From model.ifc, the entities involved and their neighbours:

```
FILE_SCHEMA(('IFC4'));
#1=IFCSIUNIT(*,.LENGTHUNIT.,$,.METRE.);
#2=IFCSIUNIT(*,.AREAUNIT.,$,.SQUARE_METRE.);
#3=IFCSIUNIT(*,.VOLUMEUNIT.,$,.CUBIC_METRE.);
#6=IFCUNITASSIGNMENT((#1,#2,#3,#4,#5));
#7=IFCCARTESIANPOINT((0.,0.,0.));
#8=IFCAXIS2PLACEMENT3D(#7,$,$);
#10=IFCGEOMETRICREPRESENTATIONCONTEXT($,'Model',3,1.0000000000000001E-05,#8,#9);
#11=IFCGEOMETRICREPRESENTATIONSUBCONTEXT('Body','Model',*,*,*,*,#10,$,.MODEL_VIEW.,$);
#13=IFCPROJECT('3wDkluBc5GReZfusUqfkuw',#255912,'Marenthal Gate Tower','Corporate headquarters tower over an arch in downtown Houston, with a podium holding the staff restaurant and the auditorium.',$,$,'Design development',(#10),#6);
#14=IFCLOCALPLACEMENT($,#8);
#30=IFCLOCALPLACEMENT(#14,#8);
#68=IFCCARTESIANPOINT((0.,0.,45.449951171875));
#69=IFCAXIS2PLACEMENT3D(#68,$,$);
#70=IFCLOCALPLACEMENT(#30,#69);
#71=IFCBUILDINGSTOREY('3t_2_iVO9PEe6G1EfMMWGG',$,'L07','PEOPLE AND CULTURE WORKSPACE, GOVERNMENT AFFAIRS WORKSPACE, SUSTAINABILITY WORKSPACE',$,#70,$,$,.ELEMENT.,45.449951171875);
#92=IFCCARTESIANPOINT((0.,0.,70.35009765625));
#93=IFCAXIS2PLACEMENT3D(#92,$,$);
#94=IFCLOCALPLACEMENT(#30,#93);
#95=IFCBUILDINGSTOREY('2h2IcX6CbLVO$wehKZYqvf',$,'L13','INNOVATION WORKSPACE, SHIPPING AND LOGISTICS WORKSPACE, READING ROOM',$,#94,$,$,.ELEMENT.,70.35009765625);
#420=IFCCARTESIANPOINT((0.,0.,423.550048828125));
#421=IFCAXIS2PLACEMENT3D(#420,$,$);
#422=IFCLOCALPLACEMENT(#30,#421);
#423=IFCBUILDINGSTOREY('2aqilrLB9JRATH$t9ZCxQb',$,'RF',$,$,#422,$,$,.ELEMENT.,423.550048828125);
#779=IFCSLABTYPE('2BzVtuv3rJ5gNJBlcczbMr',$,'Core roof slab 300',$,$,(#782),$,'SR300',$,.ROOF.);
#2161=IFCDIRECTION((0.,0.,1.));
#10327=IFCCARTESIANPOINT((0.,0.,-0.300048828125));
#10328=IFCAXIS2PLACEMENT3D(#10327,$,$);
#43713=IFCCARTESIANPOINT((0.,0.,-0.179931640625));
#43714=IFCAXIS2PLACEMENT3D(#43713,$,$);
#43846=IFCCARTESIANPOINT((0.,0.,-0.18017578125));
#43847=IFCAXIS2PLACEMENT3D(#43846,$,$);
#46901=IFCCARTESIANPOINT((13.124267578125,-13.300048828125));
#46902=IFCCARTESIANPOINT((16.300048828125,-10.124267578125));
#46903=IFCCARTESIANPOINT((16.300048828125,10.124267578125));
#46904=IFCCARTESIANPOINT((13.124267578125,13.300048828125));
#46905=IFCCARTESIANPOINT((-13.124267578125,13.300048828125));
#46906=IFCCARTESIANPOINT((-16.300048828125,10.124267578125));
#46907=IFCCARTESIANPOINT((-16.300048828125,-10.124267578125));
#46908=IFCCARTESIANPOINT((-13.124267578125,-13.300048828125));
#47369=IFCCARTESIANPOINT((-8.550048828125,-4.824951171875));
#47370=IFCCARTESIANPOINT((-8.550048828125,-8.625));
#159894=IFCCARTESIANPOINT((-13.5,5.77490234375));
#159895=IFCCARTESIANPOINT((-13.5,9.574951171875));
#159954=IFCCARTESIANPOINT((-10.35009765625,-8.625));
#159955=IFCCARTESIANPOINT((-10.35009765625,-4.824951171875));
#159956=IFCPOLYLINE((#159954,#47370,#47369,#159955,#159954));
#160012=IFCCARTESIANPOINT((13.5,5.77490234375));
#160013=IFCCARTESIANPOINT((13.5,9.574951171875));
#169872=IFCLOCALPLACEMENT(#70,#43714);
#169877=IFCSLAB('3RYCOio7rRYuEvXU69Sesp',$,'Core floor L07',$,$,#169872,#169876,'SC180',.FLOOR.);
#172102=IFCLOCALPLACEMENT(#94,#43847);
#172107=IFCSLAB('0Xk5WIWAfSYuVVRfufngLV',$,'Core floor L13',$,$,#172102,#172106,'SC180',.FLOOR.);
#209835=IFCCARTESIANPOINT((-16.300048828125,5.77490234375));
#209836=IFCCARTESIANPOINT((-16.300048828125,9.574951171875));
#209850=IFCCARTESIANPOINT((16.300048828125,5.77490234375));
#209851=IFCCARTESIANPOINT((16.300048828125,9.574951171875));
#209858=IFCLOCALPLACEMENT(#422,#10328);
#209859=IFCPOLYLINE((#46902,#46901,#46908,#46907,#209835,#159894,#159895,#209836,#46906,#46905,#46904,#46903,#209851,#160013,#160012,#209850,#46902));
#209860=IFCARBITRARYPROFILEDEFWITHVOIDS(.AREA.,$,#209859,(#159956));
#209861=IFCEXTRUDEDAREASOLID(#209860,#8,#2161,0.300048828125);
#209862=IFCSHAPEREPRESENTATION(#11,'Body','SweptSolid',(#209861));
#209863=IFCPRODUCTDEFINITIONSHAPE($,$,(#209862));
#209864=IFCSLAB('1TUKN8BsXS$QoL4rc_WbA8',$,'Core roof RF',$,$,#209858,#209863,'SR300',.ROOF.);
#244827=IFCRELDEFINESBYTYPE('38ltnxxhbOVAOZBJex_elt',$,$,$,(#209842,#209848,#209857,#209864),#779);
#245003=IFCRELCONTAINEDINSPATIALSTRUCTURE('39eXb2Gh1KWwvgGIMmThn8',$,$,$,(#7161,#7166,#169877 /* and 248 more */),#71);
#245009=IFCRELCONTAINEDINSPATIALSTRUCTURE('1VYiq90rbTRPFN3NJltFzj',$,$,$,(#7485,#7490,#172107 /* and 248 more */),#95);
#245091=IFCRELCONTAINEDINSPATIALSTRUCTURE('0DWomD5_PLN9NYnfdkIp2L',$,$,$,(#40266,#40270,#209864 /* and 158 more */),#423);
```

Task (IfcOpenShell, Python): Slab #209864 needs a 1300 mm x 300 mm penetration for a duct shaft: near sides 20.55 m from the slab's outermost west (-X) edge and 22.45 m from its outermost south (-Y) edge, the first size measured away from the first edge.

```python
import numpy as np
import ifcopenshell
import ifcopenshell.api.feature
import ifcopenshell.api.geometry
import ifcopenshell.api.root
import ifcopenshell.geom
import ifcopenshell.util.placement
import ifcopenshell.util.representation
import ifcopenshell.util.shape
import ifcopenshell.util.unit

model = ifcopenshell.open("model.ifc")
unit_scale = ifcopenshell.util.unit.calculate_unit_scale(model)
settings = ifcopenshell.geom.settings()


def volume(element):
    """Net volume in cubic metres, openings subtracted."""
    shape = ifcopenshell.geom.create_shape(settings, element)
    return ifcopenshell.util.shape.get_volume(shape.geometry)


slab = model.by_guid("1TUKN8BsXS$QoL4rc_WbA8")
before = volume(slab)

# Extent in the slab's own axes, in metres. The edges named are its -X and -Y sides.
slab_shape = ifcopenshell.geom.create_shape(settings, slab)
vertices = ifcopenshell.util.shape.get_vertices(slab_shape.geometry)
x_min, y_min, bottom = vertices.min(axis=0)
top = vertices[:, 2].max()

opening = ifcopenshell.api.root.create_entity(model, ifc_class="IfcOpeningElement", name="Duct shaft opening", predefined_type="OPENING")
context = ifcopenshell.util.representation.get_context(model, "Model", "Body", "MODEL_VIEW")
width, depth = 1.3, 0.3
outline = [(0.0, 0.0), (width, 0.0), (width, depth), (0.0, depth), (0.0, 0.0)]
# Overshoot both faces by 50 mm so the cut is clean.
shape = ifcopenshell.api.geometry.add_slab_representation(
    model, context=context, depth=top - bottom + 0.1, polyline=outline
)
ifcopenshell.api.geometry.assign_representation(model, product=opening, representation=shape)

matrix = ifcopenshell.util.placement.get_local_placement(slab.ObjectPlacement)
matrix[:, 3] = matrix @ np.append(np.array([x_min + 20.55, y_min + 22.45, bottom - 0.05]) / unit_scale, 1.0)
ifcopenshell.api.geometry.edit_object_placement(model, product=opening, matrix=matrix, is_si=False)
ifcopenshell.api.feature.add_feature(model, feature=opening, element=slab)

after = volume(slab)

print(f"slab volume {before:.3f} -> {after:.3f} m3")

model.write("model_rev.ifc")
```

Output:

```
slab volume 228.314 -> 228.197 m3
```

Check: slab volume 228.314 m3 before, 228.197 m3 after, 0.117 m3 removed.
